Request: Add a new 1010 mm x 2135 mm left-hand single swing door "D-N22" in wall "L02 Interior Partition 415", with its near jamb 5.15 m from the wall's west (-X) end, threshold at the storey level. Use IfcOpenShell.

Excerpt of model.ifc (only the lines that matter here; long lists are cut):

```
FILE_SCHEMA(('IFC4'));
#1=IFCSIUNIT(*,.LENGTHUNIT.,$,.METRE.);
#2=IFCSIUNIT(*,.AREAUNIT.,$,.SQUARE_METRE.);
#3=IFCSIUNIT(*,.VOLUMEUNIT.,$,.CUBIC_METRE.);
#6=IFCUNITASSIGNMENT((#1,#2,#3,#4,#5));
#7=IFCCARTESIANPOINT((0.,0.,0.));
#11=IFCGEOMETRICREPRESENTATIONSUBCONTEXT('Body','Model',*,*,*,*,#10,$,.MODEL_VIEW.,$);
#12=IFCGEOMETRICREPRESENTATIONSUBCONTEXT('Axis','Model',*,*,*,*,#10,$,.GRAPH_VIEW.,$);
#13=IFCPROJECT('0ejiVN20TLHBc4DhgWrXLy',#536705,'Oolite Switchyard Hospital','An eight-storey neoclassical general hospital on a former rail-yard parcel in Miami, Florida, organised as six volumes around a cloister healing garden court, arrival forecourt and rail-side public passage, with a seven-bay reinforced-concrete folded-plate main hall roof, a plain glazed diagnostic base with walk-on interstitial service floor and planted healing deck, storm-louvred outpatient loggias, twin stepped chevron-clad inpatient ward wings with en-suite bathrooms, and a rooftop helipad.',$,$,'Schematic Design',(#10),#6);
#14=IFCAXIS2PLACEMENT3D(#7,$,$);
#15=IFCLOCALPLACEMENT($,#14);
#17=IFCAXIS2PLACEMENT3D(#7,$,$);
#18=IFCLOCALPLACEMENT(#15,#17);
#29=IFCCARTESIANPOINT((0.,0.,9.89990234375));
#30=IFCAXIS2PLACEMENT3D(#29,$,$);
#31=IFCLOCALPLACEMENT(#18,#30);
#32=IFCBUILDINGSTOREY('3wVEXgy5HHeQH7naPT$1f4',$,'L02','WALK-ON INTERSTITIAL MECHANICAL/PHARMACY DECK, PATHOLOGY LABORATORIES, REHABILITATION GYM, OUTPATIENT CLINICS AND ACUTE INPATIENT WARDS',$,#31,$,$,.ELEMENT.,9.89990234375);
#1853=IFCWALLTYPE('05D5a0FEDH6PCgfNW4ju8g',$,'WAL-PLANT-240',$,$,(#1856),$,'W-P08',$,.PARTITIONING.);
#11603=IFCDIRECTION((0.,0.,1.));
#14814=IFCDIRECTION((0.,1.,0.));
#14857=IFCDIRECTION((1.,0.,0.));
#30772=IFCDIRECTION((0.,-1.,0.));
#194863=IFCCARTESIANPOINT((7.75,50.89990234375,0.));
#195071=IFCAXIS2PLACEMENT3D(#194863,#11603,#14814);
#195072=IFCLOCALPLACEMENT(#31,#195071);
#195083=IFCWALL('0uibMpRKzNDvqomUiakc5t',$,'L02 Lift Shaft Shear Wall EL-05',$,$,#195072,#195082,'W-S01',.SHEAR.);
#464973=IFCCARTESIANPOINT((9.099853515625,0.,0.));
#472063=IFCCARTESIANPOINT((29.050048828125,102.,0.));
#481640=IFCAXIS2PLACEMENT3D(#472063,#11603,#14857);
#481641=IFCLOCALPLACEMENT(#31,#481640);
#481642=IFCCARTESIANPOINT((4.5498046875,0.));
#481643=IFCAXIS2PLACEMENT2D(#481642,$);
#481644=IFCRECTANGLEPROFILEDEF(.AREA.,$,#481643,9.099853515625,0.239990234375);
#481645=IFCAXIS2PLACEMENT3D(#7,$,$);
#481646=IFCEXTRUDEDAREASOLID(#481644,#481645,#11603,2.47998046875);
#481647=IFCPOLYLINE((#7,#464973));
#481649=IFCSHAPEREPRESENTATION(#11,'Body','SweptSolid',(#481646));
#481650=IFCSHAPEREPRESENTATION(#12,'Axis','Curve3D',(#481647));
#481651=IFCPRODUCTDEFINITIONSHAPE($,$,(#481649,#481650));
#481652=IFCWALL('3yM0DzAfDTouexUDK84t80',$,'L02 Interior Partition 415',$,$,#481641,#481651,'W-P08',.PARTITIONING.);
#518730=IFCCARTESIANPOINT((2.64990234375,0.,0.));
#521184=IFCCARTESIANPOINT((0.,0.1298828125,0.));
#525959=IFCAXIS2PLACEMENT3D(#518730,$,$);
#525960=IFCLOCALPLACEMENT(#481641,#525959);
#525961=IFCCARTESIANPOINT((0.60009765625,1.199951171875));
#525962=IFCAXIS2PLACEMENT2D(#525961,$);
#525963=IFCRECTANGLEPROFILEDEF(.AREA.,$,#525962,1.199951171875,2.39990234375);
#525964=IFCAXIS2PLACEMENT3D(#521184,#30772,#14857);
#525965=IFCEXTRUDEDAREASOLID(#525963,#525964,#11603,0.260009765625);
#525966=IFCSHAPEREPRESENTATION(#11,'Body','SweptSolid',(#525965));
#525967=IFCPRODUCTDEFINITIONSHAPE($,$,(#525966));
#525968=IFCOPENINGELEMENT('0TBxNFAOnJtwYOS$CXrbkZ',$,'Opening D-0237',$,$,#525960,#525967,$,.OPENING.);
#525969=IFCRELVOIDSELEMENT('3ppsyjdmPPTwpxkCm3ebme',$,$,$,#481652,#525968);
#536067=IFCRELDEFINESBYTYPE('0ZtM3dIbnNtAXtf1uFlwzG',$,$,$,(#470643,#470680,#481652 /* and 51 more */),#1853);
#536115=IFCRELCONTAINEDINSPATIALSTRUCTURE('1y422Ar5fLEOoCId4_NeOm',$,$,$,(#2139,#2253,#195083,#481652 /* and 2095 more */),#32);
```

```python
import numpy as np
import ifcopenshell
import ifcopenshell.api.feature
import ifcopenshell.api.geometry
import ifcopenshell.api.root
import ifcopenshell.api.spatial
import ifcopenshell.geom
import ifcopenshell.util.element
import ifcopenshell.util.placement
import ifcopenshell.util.representation
import ifcopenshell.util.shape
import ifcopenshell.util.unit

model = ifcopenshell.open("model.ifc")
unit_scale = ifcopenshell.util.unit.calculate_unit_scale(model)
settings = ifcopenshell.geom.settings()


def volume(element):
    """Net volume in cubic metres, openings subtracted."""
    shape = ifcopenshell.geom.create_shape(settings, element)
    return ifcopenshell.util.shape.get_volume(shape.geometry)


wall = model.by_id(481652)
storey = ifcopenshell.util.element.get_container(wall, ifc_class="IfcBuildingStorey")
context = ifcopenshell.util.representation.get_context(model, "Model", "Body", "MODEL_VIEW")
before = volume(wall)

width, height, from_end, sill = 1.01, 2.135, 5.15, 0.0  # metres

# The wall runs along its own X axis, and the end named is its -X end.
wall_shape = ifcopenshell.geom.create_shape(settings, wall)
x, y, z = ifcopenshell.util.shape.get_vertices(wall_shape.geometry).T
start = x.min() + from_end
face, thickness = float(y.min()), float(y.max() - y.min())
wall_matrix = ifcopenshell.util.placement.get_local_placement(wall.ObjectPlacement)
level = ifcopenshell.util.placement.get_local_placement(storey.ObjectPlacement)[2, 3]


def in_wall(x, y):
    """Placement at x, y metres in the wall's axes, at sill height."""
    matrix = wall_matrix.copy()
    matrix[:, 3] = wall_matrix @ np.array([x / unit_scale, y / unit_scale, 0.0, 1.0])
    matrix[2, 3] = level + sill / unit_scale
    return matrix


# Opening: a box that overshoots both wall faces by 50 mm.
opening = ifcopenshell.api.root.create_entity(model, ifc_class="IfcOpeningElement", predefined_type="OPENING")
box = ifcopenshell.api.geometry.add_wall_representation(
    model, context=context, length=width, height=height, thickness=thickness + 0.1
)
ifcopenshell.api.geometry.assign_representation(model, product=opening, representation=box)
ifcopenshell.api.geometry.edit_object_placement(model, product=opening, matrix=in_wall(start, face - 0.05), is_si=False)
ifcopenshell.api.feature.add_feature(model, feature=opening, element=wall)

door = ifcopenshell.api.root.create_entity(model, ifc_class="IfcDoor", name="D-N22", predefined_type="DOOR")
door.OverallWidth, door.OverallHeight = width / unit_scale, height / unit_scale
door.OperationType = "SINGLE_SWING_LEFT"
body = ifcopenshell.api.geometry.add_door_representation(
    model,
    context=context,
    overall_width=door.OverallWidth,
    overall_height=door.OverallHeight,
    operation_type="SINGLE_SWING_LEFT",
    lining_properties={"LiningDepth": thickness / unit_scale, "ThresholdDepth": thickness / unit_scale},
)
ifcopenshell.api.geometry.assign_representation(model, product=door, representation=body)
ifcopenshell.api.spatial.assign_container(model, products=[door], relating_structure=storey)
ifcopenshell.api.feature.add_filling(model, opening=opening, element=door)

# The lining spans the wall, so the door starts at the wall face.
ifcopenshell.api.geometry.edit_object_placement(model, product=door, matrix=in_wall(start, face), is_si=False)

after = volume(wall)

print(f"wall volume {before:.3f} -> {after:.3f} m3")

model.write("model_v2.ifc")
```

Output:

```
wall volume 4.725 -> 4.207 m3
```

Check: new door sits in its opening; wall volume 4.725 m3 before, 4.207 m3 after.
